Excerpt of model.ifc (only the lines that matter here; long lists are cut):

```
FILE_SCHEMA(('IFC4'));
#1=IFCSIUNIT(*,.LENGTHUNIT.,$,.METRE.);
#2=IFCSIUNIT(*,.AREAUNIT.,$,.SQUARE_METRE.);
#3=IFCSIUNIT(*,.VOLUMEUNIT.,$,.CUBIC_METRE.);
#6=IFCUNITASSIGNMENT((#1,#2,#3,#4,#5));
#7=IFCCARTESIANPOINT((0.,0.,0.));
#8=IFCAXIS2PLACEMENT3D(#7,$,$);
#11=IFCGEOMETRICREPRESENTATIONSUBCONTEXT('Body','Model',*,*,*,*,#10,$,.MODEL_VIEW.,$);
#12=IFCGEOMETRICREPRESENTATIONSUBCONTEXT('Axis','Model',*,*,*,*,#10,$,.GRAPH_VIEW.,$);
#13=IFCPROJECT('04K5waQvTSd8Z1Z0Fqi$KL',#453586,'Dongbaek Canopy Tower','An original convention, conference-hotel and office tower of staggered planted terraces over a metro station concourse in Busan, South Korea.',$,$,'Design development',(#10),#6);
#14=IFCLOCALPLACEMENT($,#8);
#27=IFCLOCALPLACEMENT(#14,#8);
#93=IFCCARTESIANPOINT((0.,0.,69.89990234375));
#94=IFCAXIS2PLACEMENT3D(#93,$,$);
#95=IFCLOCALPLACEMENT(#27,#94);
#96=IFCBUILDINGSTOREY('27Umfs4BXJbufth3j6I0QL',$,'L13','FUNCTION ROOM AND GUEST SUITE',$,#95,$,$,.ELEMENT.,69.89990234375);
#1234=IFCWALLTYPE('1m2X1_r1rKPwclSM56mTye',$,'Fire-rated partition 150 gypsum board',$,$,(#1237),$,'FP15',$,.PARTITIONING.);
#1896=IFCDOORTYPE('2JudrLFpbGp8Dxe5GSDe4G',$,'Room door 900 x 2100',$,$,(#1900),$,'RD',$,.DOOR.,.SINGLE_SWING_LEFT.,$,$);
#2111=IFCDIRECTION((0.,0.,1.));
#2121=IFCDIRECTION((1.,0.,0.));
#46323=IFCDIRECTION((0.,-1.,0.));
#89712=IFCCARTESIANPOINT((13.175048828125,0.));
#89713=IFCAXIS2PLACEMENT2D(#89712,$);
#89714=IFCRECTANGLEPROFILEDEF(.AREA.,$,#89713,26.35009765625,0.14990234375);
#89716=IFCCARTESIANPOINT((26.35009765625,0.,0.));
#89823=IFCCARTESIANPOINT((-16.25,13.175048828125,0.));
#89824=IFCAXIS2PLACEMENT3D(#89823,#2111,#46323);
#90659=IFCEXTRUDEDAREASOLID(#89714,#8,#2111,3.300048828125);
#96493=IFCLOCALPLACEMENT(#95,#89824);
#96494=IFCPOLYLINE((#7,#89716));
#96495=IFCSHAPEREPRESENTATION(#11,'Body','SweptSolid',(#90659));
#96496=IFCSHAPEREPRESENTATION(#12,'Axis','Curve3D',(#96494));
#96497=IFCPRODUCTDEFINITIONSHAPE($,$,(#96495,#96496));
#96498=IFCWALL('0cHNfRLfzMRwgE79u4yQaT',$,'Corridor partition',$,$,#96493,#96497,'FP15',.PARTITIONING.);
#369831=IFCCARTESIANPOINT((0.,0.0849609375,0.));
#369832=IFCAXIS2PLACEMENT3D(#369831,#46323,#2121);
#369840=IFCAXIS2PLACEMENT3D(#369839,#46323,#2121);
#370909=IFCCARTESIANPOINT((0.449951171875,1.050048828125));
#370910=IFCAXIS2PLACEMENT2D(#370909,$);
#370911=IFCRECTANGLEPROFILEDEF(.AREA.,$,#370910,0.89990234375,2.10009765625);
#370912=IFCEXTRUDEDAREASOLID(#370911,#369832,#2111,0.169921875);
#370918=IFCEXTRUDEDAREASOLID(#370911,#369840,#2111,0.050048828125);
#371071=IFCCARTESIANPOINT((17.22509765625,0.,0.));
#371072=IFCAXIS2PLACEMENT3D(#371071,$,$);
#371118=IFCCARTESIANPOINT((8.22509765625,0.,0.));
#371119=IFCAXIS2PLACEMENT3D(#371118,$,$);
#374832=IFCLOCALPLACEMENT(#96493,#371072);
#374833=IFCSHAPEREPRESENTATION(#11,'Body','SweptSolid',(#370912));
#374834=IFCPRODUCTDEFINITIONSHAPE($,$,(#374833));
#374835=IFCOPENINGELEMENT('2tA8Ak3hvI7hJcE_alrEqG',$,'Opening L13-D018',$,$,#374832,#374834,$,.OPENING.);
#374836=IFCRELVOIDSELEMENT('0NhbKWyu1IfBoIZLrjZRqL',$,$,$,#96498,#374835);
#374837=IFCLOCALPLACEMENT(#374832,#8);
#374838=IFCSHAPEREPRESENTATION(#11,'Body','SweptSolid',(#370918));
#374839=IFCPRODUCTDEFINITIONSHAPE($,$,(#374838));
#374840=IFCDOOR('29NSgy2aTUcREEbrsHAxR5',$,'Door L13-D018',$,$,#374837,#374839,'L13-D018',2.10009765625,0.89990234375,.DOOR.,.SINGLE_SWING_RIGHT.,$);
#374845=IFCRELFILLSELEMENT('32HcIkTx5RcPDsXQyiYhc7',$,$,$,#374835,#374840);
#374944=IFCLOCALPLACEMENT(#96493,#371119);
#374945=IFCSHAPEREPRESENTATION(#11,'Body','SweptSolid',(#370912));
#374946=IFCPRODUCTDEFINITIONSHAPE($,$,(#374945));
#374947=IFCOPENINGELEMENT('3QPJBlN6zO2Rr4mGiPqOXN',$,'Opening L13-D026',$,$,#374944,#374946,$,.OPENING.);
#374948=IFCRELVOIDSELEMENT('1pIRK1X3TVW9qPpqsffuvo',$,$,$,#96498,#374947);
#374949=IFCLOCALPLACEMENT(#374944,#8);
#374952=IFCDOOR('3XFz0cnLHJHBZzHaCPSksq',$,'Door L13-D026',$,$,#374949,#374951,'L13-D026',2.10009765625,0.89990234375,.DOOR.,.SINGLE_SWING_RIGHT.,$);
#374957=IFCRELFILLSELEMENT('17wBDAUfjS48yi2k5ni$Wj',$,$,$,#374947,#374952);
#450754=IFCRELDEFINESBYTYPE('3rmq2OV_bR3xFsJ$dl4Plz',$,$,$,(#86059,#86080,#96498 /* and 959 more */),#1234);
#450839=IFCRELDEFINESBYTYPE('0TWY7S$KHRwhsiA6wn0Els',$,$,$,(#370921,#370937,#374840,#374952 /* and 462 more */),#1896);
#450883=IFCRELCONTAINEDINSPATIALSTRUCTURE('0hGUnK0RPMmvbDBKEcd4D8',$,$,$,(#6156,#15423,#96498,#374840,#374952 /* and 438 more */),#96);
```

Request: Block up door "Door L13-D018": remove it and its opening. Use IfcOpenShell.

```python
import ifcopenshell
import ifcopenshell.api.feature
import ifcopenshell.api.root
import ifcopenshell.geom
import ifcopenshell.util.shape

model = ifcopenshell.open("model.ifc")
settings = ifcopenshell.geom.settings()


def volume(element):
    """Net volume in cubic metres, openings subtracted."""
    shape = ifcopenshell.geom.create_shape(settings, element)
    return ifcopenshell.util.shape.get_volume(shape.geometry)


door = model.by_guid("29NSgy2aTUcREEbrsHAxR5")
opening = door.FillsVoids[0].RelatingOpeningElement
wall = opening.VoidsElements[0].RelatingBuildingElement
before = volume(wall)

ifcopenshell.api.root.remove_product(model, product=door)
ifcopenshell.api.feature.remove_feature(model, feature=opening)

after = volume(wall)

print(f"wall volume {before:.3f} -> {after:.3f} m3")

model.write("model_updated.ifc")
```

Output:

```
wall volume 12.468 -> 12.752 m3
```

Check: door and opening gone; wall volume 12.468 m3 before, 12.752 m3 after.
